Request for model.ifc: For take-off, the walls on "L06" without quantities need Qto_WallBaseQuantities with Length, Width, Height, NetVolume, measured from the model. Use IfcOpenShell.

First a look at what the model holds.

```python
import ifcopenshell
import ifcopenshell.util.element
import ifcopenshell.util.unit

model = ifcopenshell.open("model.ifc")
print(model.schema)
for unit_type in ("LENGTHUNIT", "AREAUNIT", "VOLUMEUNIT"):
    print(unit_type, ifcopenshell.util.unit.calculate_unit_scale(model, unit_type))
storey = next(s for s in model.by_type("IfcBuildingStorey") if s.Name == "L06")
walls = [e for e in ifcopenshell.util.element.get_decomposition(storey) if e.is_a("IfcWall")]
for e in sorted(walls, key=lambda e: e.id()):
    print(e.id(), e.is_a(), e.Name, list(ifcopenshell.util.element.get_psets(e, qtos_only=True)), sep=" | ")
```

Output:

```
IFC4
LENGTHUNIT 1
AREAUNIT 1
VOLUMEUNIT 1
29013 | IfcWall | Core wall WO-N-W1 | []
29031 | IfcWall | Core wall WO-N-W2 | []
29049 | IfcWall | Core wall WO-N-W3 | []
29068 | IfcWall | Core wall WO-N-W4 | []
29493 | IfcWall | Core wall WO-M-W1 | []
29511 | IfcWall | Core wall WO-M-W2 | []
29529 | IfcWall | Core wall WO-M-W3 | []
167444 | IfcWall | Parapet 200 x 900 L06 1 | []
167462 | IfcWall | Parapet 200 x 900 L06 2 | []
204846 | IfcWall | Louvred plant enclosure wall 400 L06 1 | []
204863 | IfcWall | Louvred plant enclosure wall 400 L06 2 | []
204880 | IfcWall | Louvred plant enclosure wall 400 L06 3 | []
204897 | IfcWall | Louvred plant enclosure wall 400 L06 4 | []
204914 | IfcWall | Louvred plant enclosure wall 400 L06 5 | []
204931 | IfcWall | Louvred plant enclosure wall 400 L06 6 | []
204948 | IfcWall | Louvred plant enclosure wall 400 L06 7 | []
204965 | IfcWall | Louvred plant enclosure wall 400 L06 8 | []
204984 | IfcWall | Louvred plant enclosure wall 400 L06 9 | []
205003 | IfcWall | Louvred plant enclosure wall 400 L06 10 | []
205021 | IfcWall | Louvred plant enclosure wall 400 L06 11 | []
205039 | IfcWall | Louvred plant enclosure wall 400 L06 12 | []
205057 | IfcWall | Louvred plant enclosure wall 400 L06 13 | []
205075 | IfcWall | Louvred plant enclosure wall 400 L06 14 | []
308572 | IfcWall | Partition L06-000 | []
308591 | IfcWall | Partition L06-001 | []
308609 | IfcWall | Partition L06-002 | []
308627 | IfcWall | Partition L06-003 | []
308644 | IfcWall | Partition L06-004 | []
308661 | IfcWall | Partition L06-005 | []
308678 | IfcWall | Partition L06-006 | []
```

```python
import ifcopenshell
import ifcopenshell.api.pset
import ifcopenshell.geom
import ifcopenshell.util.element
import ifcopenshell.util.shape
import ifcopenshell.util.unit

model = ifcopenshell.open("model.ifc")
unit_scale = ifcopenshell.util.unit.calculate_unit_scale(model)
volume_scale = ifcopenshell.util.unit.calculate_unit_scale(model, "VOLUMEUNIT")
settings = ifcopenshell.geom.settings()

storey = next(s for s in model.by_type("IfcBuildingStorey") if s.Name == "L06")
walls = [e for e in ifcopenshell.util.element.get_decomposition(storey) if e.is_a("IfcWall")]

for e in sorted(walls, key=lambda e: e.id()):
    if ifcopenshell.util.element.get_psets(e, qtos_only=True, should_inherit=False):
        continue
    # Geometry comes back in metres, in the element's own axes.
    shape = ifcopenshell.geom.create_shape(settings, e)
    values = {
        "Length": ifcopenshell.util.shape.get_x(shape.geometry) / unit_scale,
        "Width": ifcopenshell.util.shape.get_y(shape.geometry) / unit_scale,
        "Height": ifcopenshell.util.shape.get_z(shape.geometry) / unit_scale,
        "NetVolume": ifcopenshell.util.shape.get_volume(shape.geometry) / volume_scale,
    }
    qto = ifcopenshell.api.pset.add_qto(model, product=e, name="Qto_WallBaseQuantities")
    ifcopenshell.api.pset.edit_qto(model, qto=qto, properties=values)
    print(e.id(), {k: round(v, 3) for k, v in values.items()})

model.write("model_edited.ifc")
```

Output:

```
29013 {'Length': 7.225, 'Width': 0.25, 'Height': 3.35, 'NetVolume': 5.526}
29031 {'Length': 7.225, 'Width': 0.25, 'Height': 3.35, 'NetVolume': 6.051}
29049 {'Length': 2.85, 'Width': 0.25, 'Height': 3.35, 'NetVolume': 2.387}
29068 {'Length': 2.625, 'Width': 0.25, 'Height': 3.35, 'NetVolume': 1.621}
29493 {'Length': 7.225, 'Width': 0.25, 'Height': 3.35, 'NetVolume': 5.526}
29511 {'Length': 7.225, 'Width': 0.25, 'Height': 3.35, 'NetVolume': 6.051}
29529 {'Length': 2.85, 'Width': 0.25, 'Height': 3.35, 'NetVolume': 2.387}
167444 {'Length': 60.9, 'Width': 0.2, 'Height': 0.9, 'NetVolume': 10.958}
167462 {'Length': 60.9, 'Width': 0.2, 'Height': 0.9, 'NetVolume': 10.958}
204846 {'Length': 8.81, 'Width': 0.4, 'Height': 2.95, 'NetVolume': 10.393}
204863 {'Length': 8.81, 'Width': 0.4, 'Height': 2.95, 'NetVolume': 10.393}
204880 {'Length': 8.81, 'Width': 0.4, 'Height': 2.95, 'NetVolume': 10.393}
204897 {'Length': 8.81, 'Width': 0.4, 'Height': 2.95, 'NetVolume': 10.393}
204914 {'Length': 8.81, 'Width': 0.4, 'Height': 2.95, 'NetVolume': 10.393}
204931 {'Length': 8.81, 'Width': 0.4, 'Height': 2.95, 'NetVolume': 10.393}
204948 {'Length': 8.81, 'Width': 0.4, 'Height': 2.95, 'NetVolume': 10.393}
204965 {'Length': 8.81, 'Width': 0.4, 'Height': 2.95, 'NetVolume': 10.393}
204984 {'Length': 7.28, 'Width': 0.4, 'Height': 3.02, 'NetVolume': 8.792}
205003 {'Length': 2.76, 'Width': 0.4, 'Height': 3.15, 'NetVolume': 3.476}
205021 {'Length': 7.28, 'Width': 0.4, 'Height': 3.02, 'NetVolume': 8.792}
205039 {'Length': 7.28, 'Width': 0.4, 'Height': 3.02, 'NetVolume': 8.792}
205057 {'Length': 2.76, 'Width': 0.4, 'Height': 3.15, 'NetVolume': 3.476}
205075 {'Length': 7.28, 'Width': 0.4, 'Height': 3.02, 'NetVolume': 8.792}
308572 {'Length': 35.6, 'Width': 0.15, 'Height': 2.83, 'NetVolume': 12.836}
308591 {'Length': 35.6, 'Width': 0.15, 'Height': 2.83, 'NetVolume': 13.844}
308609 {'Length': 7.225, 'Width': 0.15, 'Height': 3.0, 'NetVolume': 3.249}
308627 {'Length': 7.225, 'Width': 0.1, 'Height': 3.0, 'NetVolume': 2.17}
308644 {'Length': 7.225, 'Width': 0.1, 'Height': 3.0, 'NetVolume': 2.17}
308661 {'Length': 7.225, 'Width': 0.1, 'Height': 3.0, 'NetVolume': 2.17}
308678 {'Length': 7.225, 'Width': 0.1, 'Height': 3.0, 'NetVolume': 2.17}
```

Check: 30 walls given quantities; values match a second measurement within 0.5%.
